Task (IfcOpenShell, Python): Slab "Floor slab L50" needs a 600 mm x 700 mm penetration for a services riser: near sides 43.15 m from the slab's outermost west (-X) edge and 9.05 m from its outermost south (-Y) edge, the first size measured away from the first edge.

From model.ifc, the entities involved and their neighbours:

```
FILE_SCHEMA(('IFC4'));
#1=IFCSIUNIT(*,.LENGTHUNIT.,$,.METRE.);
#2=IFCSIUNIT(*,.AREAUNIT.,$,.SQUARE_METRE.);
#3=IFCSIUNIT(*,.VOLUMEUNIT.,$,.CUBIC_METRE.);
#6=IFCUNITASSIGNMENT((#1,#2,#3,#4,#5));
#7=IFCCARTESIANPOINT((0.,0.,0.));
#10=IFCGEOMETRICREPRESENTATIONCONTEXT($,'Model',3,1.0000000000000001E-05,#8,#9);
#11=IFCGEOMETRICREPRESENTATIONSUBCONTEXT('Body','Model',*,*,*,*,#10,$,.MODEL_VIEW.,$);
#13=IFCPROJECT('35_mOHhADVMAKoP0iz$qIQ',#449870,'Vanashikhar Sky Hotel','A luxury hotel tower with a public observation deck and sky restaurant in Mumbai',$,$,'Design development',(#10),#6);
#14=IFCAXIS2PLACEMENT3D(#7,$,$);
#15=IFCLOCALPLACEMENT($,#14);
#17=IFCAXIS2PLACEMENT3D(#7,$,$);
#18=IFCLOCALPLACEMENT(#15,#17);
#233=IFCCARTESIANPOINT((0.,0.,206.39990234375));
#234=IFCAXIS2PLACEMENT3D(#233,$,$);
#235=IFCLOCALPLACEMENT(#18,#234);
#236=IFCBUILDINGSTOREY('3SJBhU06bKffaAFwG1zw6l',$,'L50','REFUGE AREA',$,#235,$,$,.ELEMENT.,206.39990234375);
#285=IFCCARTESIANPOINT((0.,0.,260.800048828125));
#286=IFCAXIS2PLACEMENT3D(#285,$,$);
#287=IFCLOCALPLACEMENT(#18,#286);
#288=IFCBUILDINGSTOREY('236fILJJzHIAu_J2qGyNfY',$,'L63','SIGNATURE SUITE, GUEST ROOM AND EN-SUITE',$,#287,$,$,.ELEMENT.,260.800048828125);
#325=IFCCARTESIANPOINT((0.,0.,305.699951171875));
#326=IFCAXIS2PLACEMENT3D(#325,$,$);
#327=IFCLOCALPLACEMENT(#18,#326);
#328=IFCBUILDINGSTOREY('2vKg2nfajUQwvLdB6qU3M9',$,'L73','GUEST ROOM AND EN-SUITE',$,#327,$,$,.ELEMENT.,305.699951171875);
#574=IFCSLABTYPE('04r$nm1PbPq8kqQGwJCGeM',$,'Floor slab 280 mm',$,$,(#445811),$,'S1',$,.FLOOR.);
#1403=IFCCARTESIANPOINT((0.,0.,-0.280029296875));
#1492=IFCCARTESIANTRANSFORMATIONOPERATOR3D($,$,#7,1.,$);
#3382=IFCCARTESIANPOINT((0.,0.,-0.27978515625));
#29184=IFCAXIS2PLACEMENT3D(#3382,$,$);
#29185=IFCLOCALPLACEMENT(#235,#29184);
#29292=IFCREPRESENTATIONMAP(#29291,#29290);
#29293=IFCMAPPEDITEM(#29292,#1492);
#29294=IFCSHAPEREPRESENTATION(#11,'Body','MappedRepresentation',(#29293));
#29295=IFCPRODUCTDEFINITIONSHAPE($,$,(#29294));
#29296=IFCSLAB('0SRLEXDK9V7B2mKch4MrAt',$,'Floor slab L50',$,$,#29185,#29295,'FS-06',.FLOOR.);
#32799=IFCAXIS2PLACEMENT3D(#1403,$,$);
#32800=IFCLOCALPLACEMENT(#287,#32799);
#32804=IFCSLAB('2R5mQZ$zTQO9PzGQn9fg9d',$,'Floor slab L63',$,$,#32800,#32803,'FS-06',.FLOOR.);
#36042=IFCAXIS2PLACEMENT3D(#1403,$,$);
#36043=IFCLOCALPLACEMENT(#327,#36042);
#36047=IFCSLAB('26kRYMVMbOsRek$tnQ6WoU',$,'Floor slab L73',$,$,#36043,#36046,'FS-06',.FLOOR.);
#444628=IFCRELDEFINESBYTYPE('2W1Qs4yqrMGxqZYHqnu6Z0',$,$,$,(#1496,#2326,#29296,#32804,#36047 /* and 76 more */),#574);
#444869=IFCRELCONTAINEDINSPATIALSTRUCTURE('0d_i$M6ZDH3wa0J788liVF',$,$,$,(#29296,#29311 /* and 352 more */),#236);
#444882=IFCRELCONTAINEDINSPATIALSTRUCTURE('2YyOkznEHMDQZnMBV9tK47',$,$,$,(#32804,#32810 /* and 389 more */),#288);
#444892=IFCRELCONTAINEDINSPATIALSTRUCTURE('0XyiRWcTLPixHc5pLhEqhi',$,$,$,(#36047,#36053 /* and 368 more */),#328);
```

```python
import numpy as np
import ifcopenshell
import ifcopenshell.api.feature
import ifcopenshell.api.geometry
import ifcopenshell.api.root
import ifcopenshell.geom
import ifcopenshell.util.placement
import ifcopenshell.util.representation
import ifcopenshell.util.shape
import ifcopenshell.util.unit

model = ifcopenshell.open("model.ifc")
unit_scale = ifcopenshell.util.unit.calculate_unit_scale(model)
settings = ifcopenshell.geom.settings()


def volume(element):
    """Net volume in cubic metres, openings subtracted."""
    shape = ifcopenshell.geom.create_shape(settings, element)
    return ifcopenshell.util.shape.get_volume(shape.geometry)


slab = model.by_guid("0SRLEXDK9V7B2mKch4MrAt")
before = volume(slab)

# Extent in the slab's own axes, in metres. The edges named are its -X and -Y sides.
slab_shape = ifcopenshell.geom.create_shape(settings, slab)
vertices = ifcopenshell.util.shape.get_vertices(slab_shape.geometry)
x_min, y_min, bottom = vertices.min(axis=0)
top = vertices[:, 2].max()

opening = ifcopenshell.api.root.create_entity(model, ifc_class="IfcOpeningElement", name="Services riser opening", predefined_type="OPENING")
context = ifcopenshell.util.representation.get_context(model, "Model", "Body", "MODEL_VIEW")
width, depth = 0.6, 0.7
outline = [(0.0, 0.0), (width, 0.0), (width, depth), (0.0, depth), (0.0, 0.0)]
# Overshoot both faces by 50 mm so the cut is clean.
shape = ifcopenshell.api.geometry.add_slab_representation(
    model, context=context, depth=top - bottom + 0.1, polyline=outline
)
ifcopenshell.api.geometry.assign_representation(model, product=opening, representation=shape)

matrix = ifcopenshell.util.placement.get_local_placement(slab.ObjectPlacement)
matrix[:, 3] = matrix @ np.append(np.array([x_min + 43.15, y_min + 9.05, bottom - 0.05]) / unit_scale, 1.0)
ifcopenshell.api.geometry.edit_object_placement(model, product=opening, matrix=matrix, is_si=False)
ifcopenshell.api.feature.add_feature(model, feature=opening, element=slab)

after = volume(slab)

print(f"slab volume {before:.3f} -> {after:.3f} m3")

model.write("model-out.ifc")
```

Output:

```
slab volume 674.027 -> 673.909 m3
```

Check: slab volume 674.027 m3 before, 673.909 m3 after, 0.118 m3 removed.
